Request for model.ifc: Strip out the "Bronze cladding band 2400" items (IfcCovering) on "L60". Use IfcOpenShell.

First a look at what the model holds.

```python
import ifcopenshell
import ifcopenshell.util.element

model = ifcopenshell.open("model.ifc")
print(model.schema)
storey = next(s for s in model.by_type("IfcBuildingStorey") if s.Name == "L60")
coverings = [e for e in ifcopenshell.util.element.get_decomposition(storey) if e.is_a("IfcCovering")]
seen = {}
for e in coverings:
    element_type = ifcopenshell.util.element.get_type(e)
    name = element_type.Name if element_type not in (None, e) else None
    seen[name] = seen.get(name, 0) + 1
for name, count in sorted(seen.items(), key=str):
    print(count, "x", name)
```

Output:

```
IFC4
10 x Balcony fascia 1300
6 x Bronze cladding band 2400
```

```python
import ifcopenshell
import ifcopenshell.api.root
import ifcopenshell.util.element

model = ifcopenshell.open("model.ifc")

storey = next(s for s in model.by_type("IfcBuildingStorey") if s.Name == "L60")
coverings = [e for e in ifcopenshell.util.element.get_decomposition(storey) if e.is_a("IfcCovering")]
targets = [e for e in coverings if (t := ifcopenshell.util.element.get_type(e)) not in (None, e) and t.Name == "Bronze cladding band 2400"]

for e in targets:
    ifcopenshell.api.root.remove_product(model, product=e)
print(len(targets), "removed")

model.write("model_rev.ifc")
```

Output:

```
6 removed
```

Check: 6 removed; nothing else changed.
